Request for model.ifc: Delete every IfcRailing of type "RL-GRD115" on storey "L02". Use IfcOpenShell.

First a look at what the model holds.

```python
import ifcopenshell
import ifcopenshell.util.element

model = ifcopenshell.open("model.ifc")
print(model.schema)
storey = next(s for s in model.by_type("IfcBuildingStorey") if s.Name == "L02")
railings = [e for e in ifcopenshell.util.element.get_decomposition(storey) if e.is_a("IfcRailing")]
seen = {}
for e in railings:
    element_type = ifcopenshell.util.element.get_type(e)
    name = element_type.Name if element_type not in (None, e) else None
    seen[name] = seen.get(name, 0) + 1
for name, count in sorted(seen.items(), key=str):
    print(count, "x", name)
```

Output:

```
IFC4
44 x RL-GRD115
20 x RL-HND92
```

```python
import ifcopenshell
import ifcopenshell.api.root
import ifcopenshell.util.element

model = ifcopenshell.open("model.ifc")

storey = next(s for s in model.by_type("IfcBuildingStorey") if s.Name == "L02")
railings = [e for e in ifcopenshell.util.element.get_decomposition(storey) if e.is_a("IfcRailing")]
targets = [e for e in railings if (t := ifcopenshell.util.element.get_type(e)) not in (None, e) and t.Name == "RL-GRD115"]

for e in targets:
    ifcopenshell.api.root.remove_product(model, product=e)
print(len(targets), "removed")

model.write("model_rev.ifc")
```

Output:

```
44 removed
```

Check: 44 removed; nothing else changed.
